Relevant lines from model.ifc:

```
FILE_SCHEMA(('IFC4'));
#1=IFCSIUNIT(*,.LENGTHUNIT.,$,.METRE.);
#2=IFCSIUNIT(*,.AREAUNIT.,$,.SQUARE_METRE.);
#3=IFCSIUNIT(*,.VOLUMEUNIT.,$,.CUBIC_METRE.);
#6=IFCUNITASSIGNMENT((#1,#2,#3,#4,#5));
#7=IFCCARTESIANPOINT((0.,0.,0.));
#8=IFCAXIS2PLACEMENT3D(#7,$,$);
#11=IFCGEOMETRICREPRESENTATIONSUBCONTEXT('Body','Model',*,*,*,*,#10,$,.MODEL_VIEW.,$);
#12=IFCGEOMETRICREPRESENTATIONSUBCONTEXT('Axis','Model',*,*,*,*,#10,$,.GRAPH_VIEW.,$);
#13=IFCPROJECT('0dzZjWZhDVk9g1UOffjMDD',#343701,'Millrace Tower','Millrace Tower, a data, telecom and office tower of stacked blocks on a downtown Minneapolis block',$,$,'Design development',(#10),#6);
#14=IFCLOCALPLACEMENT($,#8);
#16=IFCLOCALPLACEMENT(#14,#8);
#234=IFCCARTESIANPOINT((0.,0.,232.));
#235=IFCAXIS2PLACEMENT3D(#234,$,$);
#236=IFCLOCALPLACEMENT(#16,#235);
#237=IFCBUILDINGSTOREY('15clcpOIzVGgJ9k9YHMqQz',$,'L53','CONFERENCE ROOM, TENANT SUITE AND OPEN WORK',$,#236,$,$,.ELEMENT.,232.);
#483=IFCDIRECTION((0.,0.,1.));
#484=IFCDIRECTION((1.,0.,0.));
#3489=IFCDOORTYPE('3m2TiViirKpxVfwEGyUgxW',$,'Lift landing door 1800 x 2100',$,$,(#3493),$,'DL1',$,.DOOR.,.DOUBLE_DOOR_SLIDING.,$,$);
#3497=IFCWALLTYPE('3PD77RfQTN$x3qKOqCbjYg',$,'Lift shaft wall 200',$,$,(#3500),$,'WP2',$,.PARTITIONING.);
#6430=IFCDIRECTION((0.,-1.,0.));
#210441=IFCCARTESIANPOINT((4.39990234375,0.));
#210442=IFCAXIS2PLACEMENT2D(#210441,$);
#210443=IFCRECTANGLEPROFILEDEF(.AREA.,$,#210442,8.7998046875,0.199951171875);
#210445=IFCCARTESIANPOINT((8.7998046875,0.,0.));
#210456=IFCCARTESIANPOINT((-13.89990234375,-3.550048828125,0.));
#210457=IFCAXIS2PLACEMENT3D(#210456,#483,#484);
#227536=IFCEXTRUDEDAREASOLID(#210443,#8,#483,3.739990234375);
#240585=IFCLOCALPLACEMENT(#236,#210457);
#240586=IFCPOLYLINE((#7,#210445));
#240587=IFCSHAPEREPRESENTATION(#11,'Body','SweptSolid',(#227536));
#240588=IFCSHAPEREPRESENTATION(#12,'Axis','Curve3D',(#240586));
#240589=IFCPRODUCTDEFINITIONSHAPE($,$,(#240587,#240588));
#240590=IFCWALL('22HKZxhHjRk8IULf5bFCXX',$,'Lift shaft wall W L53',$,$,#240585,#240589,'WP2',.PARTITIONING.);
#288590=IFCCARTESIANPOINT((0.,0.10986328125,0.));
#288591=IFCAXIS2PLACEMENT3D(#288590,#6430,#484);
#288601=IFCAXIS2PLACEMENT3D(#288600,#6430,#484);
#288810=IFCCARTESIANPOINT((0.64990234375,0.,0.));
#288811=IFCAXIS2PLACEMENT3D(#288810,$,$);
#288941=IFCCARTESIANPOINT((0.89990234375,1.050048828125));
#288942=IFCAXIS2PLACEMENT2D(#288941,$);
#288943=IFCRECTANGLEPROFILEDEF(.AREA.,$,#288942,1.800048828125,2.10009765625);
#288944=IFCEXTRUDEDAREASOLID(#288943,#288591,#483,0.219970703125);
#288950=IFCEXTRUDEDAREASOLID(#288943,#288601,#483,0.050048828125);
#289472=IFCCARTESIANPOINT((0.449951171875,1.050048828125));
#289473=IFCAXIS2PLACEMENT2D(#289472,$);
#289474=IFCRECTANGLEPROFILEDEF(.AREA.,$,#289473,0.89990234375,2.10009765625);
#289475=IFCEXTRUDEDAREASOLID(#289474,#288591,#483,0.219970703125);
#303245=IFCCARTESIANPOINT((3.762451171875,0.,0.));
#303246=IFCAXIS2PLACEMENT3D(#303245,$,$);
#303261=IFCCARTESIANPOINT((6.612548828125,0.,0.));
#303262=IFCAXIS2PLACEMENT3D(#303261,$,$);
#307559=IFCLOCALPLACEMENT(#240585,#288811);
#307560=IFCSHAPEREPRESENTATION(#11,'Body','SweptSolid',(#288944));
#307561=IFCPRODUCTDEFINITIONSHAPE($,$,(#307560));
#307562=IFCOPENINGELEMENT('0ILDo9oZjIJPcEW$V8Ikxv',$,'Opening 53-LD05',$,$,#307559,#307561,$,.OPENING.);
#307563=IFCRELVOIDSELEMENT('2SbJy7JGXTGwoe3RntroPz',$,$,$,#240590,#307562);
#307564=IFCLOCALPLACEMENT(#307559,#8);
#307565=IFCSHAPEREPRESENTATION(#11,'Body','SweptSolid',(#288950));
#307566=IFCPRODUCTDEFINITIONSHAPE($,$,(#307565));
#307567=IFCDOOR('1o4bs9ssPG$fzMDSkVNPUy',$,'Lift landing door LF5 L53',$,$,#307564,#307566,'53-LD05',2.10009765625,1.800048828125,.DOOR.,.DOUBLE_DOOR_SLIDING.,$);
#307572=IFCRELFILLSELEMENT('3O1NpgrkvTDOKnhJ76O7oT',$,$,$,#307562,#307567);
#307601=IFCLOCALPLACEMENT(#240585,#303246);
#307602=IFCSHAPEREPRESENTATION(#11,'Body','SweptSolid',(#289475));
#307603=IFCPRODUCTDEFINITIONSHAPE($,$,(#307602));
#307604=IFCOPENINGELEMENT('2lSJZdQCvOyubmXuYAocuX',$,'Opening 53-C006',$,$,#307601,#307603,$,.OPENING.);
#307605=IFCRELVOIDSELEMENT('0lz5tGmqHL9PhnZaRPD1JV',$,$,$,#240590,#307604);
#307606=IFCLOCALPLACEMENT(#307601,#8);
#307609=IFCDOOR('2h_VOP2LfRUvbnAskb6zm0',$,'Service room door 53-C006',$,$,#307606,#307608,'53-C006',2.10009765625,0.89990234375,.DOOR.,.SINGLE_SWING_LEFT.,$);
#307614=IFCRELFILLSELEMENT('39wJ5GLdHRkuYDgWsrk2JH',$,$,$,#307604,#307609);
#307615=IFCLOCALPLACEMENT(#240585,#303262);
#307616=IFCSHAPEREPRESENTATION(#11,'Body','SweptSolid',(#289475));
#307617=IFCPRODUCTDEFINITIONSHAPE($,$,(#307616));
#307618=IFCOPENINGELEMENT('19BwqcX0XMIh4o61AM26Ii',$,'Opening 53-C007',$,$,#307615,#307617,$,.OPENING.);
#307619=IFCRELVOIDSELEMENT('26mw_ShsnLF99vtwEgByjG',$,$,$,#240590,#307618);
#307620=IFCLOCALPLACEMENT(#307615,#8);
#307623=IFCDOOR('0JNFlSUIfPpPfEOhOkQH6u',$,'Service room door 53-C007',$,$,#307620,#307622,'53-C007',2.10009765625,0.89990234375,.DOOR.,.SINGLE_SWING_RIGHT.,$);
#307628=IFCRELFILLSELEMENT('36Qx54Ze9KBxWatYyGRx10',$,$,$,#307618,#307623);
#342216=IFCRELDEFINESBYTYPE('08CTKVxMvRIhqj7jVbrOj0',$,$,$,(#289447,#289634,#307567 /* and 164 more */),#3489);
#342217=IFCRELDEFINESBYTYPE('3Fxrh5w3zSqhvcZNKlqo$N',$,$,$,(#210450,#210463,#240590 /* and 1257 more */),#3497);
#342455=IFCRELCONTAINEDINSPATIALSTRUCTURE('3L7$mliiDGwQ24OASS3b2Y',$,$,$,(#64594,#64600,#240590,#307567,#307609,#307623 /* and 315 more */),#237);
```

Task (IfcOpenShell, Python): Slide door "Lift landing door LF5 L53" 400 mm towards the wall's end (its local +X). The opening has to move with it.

```python
import ifcopenshell
import ifcopenshell.api.geometry
import ifcopenshell.util.placement

model = ifcopenshell.open("model.ifc")

door = model.by_guid("1o4bs9ssPG$fzMDSkVNPUy")
opening = door.FillsVoids[0].RelatingOpeningElement
wall = opening.VoidsElements[0].RelatingBuildingElement

wall_matrix = ifcopenshell.util.placement.get_local_placement(wall.ObjectPlacement)
shift = wall_matrix[:3, 0] * 0.4
before = ifcopenshell.util.placement.get_local_placement(door.ObjectPlacement)[:3, 3].copy()

# The door is placed relative to its opening, so it follows when the opening moves.
matrix = ifcopenshell.util.placement.get_local_placement(opening.ObjectPlacement)
matrix[:3, 3] += shift
ifcopenshell.api.geometry.edit_object_placement(
    model, product=opening, matrix=matrix, is_si=False, should_transform_children=True
)

after = ifcopenshell.util.placement.get_local_placement(door.ObjectPlacement)[:3, 3]
print("door moved by", (after - before).round(3) + 0.0)

model.write("model_updated.ifc")
```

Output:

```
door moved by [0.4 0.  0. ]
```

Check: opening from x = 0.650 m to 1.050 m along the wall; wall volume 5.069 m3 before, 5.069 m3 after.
